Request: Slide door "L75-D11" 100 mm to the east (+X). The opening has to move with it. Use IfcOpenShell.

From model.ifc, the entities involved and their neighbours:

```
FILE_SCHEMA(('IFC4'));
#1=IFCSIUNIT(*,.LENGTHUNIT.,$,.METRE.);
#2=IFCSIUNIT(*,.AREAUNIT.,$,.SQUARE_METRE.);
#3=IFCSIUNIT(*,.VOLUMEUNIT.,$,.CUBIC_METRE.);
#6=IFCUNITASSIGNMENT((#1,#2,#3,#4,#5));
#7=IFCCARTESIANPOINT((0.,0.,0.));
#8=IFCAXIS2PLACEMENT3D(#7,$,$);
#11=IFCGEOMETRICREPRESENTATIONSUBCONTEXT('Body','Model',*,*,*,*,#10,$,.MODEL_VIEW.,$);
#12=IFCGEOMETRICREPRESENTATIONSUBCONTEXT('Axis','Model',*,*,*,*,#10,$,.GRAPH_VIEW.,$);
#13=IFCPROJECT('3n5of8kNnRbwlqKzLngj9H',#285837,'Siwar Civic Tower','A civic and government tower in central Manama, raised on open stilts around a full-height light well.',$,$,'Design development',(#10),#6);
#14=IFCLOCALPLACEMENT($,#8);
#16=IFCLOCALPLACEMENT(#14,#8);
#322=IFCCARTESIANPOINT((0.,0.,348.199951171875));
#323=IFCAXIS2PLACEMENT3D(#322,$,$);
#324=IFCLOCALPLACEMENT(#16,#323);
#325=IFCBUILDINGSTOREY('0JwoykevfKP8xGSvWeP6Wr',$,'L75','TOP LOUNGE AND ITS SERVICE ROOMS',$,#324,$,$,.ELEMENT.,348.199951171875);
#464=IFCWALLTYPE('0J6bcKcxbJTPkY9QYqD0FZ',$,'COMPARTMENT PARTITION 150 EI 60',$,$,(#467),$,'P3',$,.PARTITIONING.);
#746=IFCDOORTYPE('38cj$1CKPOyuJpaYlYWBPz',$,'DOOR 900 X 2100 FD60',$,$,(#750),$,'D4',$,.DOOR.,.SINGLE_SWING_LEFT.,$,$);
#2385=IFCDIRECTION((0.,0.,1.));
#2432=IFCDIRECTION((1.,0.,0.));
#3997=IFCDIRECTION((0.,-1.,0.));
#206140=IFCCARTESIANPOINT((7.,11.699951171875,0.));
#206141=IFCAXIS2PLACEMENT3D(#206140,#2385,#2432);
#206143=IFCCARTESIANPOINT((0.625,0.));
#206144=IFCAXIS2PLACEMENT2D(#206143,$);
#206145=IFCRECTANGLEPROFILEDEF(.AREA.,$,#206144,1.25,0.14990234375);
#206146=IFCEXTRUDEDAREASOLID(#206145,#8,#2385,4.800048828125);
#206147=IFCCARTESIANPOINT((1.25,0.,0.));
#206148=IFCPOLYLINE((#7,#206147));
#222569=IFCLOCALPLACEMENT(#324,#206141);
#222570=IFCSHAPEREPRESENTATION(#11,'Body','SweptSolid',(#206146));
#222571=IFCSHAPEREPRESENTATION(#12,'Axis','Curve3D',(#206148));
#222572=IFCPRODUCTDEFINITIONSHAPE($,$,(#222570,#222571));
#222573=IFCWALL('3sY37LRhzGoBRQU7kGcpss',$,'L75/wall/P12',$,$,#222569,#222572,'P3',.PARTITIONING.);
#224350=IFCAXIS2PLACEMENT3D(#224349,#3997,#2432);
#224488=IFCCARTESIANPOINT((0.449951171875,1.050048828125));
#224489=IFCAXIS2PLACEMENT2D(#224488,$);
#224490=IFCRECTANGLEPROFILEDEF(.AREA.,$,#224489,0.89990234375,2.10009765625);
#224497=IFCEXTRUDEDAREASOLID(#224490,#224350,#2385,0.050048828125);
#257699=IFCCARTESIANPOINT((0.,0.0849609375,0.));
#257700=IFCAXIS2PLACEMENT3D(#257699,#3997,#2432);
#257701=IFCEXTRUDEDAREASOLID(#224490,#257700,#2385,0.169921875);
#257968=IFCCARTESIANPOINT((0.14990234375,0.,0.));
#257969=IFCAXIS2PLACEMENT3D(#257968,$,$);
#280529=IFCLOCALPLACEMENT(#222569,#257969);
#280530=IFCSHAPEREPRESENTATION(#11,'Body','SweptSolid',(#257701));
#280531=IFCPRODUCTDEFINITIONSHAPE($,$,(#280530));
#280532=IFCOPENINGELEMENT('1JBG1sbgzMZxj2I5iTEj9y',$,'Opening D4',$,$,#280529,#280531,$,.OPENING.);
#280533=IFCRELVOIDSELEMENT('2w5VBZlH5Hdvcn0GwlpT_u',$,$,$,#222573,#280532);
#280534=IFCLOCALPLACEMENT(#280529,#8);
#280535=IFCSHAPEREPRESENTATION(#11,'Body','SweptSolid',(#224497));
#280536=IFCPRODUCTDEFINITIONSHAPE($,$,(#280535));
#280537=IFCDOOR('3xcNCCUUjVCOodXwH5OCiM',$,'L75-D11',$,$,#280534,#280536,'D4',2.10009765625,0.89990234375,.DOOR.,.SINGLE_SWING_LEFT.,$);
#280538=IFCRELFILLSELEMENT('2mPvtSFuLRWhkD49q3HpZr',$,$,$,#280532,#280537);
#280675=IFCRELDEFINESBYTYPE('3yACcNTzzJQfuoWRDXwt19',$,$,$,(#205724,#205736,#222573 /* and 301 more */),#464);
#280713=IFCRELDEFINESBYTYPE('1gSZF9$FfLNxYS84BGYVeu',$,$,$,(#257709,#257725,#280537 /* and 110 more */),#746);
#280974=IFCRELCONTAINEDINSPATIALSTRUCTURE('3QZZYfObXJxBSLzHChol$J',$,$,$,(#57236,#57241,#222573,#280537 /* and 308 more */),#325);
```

```python
import ifcopenshell
import ifcopenshell.api.geometry
import ifcopenshell.util.placement

model = ifcopenshell.open("model.ifc")

door = model.by_guid("3xcNCCUUjVCOodXwH5OCiM")
opening = door.FillsVoids[0].RelatingOpeningElement
wall = opening.VoidsElements[0].RelatingBuildingElement

wall_matrix = ifcopenshell.util.placement.get_local_placement(wall.ObjectPlacement)
shift = wall_matrix[:3, 0] * 0.1
before = ifcopenshell.util.placement.get_local_placement(door.ObjectPlacement)[:3, 3].copy()

# The door is placed relative to its opening, so it follows when the opening moves.
matrix = ifcopenshell.util.placement.get_local_placement(opening.ObjectPlacement)
matrix[:3, 3] += shift
ifcopenshell.api.geometry.edit_object_placement(
    model, product=opening, matrix=matrix, is_si=False, should_transform_children=True
)

after = ifcopenshell.util.placement.get_local_placement(door.ObjectPlacement)[:3, 3]
print("door moved by", (after - before).round(3) + 0.0)

model.write("model-out.ifc")
```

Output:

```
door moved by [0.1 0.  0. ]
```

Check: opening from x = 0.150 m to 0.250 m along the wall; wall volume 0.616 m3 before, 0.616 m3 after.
